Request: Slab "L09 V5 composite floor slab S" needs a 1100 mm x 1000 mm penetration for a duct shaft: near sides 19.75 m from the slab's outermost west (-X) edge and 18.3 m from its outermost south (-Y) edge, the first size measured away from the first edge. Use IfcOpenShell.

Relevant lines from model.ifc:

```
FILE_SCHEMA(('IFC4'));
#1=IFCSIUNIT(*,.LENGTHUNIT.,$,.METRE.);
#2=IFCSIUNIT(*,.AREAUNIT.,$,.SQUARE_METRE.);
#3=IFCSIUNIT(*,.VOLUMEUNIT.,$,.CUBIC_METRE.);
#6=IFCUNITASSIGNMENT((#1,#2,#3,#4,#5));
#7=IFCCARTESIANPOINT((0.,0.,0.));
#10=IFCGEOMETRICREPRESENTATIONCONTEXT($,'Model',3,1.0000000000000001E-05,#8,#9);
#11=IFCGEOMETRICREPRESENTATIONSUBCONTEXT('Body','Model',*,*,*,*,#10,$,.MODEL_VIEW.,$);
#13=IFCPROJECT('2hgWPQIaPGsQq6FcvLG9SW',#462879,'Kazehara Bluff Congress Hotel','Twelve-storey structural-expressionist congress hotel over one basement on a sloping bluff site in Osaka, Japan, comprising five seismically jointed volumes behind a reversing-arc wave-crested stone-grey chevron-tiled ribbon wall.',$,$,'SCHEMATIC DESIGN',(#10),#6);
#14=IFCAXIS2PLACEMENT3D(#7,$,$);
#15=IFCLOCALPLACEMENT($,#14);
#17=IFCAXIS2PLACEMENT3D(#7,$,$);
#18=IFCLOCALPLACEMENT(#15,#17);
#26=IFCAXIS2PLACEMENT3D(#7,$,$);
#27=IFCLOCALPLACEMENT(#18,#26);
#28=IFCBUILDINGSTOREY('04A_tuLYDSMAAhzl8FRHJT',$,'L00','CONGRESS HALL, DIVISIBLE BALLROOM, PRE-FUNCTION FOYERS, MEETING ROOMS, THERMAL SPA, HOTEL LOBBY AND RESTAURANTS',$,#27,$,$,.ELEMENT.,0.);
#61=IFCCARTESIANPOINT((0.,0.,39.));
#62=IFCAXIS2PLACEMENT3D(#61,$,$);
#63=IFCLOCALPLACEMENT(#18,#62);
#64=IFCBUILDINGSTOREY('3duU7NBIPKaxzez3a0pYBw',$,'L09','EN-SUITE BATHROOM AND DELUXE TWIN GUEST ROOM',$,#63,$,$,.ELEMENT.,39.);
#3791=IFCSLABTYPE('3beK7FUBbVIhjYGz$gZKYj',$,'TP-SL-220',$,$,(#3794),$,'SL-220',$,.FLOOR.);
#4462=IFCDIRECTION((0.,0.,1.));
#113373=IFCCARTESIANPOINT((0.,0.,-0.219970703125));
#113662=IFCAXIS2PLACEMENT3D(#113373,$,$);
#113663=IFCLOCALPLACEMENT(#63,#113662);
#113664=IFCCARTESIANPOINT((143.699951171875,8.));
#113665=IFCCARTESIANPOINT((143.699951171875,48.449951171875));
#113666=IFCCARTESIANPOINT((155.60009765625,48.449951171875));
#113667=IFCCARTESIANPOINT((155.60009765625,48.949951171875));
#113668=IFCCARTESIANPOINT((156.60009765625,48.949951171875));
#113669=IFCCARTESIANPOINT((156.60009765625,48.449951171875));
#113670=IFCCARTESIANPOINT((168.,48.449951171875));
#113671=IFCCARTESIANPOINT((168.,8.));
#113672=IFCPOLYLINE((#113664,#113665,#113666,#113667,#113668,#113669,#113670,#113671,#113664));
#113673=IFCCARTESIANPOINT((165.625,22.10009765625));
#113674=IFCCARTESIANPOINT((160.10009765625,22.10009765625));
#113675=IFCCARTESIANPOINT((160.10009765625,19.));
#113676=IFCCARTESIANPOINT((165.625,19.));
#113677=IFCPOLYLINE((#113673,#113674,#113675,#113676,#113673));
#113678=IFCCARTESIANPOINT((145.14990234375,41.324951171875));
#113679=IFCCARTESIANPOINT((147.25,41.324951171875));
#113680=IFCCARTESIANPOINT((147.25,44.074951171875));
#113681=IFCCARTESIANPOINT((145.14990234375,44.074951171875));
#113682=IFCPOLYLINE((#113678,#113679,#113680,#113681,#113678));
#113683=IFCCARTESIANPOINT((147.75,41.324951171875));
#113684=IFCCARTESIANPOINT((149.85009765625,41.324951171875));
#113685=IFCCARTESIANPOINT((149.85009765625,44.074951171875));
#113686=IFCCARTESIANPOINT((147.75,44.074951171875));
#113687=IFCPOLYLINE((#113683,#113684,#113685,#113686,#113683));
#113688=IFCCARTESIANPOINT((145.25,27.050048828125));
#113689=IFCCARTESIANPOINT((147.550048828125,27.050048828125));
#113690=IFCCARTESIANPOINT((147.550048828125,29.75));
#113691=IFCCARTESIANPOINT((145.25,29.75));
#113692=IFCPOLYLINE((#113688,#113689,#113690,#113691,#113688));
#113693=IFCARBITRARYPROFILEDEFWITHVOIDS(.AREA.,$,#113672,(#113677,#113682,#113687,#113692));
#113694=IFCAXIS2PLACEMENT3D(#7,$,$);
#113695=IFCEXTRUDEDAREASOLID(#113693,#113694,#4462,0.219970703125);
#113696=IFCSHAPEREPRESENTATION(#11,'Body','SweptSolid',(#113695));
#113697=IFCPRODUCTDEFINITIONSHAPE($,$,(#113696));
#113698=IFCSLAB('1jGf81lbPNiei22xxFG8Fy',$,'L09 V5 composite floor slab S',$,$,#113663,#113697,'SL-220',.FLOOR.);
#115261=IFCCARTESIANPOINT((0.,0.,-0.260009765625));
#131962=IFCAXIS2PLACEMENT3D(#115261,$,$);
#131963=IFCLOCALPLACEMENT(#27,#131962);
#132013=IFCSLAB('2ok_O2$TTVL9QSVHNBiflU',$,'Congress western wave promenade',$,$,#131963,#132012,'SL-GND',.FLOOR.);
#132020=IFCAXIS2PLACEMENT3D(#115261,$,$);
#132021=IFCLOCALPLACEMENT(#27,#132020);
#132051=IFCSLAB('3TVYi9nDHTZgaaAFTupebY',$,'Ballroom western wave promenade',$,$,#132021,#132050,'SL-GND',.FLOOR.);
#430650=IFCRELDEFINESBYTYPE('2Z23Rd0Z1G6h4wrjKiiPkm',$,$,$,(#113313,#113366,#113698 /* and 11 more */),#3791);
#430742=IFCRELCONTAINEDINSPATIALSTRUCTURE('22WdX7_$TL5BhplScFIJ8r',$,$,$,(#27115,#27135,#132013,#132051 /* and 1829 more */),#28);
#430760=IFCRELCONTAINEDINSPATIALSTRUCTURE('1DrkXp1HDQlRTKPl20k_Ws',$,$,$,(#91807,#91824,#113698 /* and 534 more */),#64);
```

```python
import numpy as np
import ifcopenshell
import ifcopenshell.api.feature
import ifcopenshell.api.geometry
import ifcopenshell.api.root
import ifcopenshell.geom
import ifcopenshell.util.placement
import ifcopenshell.util.representation
import ifcopenshell.util.shape
import ifcopenshell.util.unit

model = ifcopenshell.open("model.ifc")
unit_scale = ifcopenshell.util.unit.calculate_unit_scale(model)
settings = ifcopenshell.geom.settings()


def volume(element):
    """Net volume in cubic metres, openings subtracted."""
    shape = ifcopenshell.geom.create_shape(settings, element)
    return ifcopenshell.util.shape.get_volume(shape.geometry)


slab = model.by_guid("1jGf81lbPNiei22xxFG8Fy")
before = volume(slab)

# Extent in the slab's own axes, in metres. The edges named are its -X and -Y sides.
slab_shape = ifcopenshell.geom.create_shape(settings, slab)
vertices = ifcopenshell.util.shape.get_vertices(slab_shape.geometry)
x_min, y_min, bottom = vertices.min(axis=0)
top = vertices[:, 2].max()

opening = ifcopenshell.api.root.create_entity(model, ifc_class="IfcOpeningElement", name="Duct shaft opening", predefined_type="OPENING")
context = ifcopenshell.util.representation.get_context(model, "Model", "Body", "MODEL_VIEW")
width, depth = 1.1, 1
outline = [(0.0, 0.0), (width, 0.0), (width, depth), (0.0, depth), (0.0, 0.0)]
# Overshoot both faces by 50 mm so the cut is clean.
shape = ifcopenshell.api.geometry.add_slab_representation(
    model, context=context, depth=top - bottom + 0.1, polyline=outline
)
ifcopenshell.api.geometry.assign_representation(model, product=opening, representation=shape)

matrix = ifcopenshell.util.placement.get_local_placement(slab.ObjectPlacement)
matrix[:, 3] = matrix @ np.append(np.array([x_min + 19.75, y_min + 18.3, bottom - 0.05]) / unit_scale, 1.0)
ifcopenshell.api.geometry.edit_object_placement(model, product=opening, matrix=matrix, is_si=False)
ifcopenshell.api.feature.add_feature(model, feature=opening, element=slab)

after = volume(slab)

print(f"slab volume {before:.3f} -> {after:.3f} m3")

model.write("model_updated.ifc")
```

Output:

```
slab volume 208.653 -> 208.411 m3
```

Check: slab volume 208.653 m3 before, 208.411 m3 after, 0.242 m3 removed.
